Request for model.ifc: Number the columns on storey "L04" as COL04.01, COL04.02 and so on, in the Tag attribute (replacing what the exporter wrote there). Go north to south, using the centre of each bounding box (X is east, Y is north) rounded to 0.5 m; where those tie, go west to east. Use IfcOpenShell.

First a look at what the model holds.

```python
import ifcopenshell
import ifcopenshell.util.element
import ifcopenshell.util.placement

model = ifcopenshell.open("model.ifc")
print(model.schema)
storey = next(s for s in model.by_type("IfcBuildingStorey") if s.Name == "L04")
columns = [e for e in ifcopenshell.util.element.get_decomposition(storey) if e.is_a("IfcColumn")]
for e in sorted(columns, key=lambda e: e.id()):
    origin = ifcopenshell.util.placement.get_local_placement(e.ObjectPlacement)[:3, 3]
    print(e.id(), e.Tag, e.Name, origin.round(2) + 0.0, sep=" | ")
```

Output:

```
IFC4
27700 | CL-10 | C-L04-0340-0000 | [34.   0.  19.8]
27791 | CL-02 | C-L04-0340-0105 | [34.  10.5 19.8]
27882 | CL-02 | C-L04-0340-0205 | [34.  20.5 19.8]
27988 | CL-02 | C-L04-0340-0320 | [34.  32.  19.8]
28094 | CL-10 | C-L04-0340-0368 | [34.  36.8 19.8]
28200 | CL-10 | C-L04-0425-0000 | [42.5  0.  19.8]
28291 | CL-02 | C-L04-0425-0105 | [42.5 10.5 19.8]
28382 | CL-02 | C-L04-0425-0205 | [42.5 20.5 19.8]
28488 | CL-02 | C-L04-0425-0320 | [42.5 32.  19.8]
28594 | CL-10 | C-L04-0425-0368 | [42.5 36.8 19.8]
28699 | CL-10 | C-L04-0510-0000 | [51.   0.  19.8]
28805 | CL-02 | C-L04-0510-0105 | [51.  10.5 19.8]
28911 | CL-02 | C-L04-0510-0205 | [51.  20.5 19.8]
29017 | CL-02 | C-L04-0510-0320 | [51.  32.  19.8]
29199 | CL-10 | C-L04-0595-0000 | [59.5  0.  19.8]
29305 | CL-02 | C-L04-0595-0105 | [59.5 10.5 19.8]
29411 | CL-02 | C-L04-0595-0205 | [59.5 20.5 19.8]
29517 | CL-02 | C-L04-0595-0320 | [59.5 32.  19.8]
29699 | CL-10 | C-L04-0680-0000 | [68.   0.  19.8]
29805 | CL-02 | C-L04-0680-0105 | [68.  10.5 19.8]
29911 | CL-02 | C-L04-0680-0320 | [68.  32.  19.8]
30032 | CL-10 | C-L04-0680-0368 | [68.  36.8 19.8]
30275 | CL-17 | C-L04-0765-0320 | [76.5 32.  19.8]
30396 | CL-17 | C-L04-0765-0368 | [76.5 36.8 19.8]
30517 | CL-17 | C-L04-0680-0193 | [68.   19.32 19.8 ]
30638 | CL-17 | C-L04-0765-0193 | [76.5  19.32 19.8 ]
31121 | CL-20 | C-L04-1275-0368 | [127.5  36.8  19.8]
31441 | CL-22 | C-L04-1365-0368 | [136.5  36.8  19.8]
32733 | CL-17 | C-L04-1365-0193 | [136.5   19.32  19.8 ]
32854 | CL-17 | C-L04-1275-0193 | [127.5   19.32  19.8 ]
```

```python
import ifcopenshell
import ifcopenshell.geom
import ifcopenshell.util.element
import ifcopenshell.util.shape

model = ifcopenshell.open("model.ifc")
settings = ifcopenshell.geom.settings()
settings.set("use-world-coords", True)


def centre(element):
    shape = ifcopenshell.geom.create_shape(settings, element)
    return ifcopenshell.util.shape.get_bbox_centroid(shape.geometry)


storey = next(s for s in model.by_type("IfcBuildingStorey") if s.Name == "L04")
columns = [e for e in ifcopenshell.util.element.get_decomposition(storey) if e.is_a("IfcColumn")]

# Insertion points can sit at a corner or the storey origin, so sort by the geometry (in metres).
centres = {e: centre(e) for e in columns}
columns.sort(key=lambda e: (-round(centres[e][1] / 0.5), centres[e][0]))

for i, e in enumerate(columns, start=1):
    number = f"COL04.{i:02d}"
    e.Tag = number
    print(e.id(), number)

model.write("model_updated.ifc")
```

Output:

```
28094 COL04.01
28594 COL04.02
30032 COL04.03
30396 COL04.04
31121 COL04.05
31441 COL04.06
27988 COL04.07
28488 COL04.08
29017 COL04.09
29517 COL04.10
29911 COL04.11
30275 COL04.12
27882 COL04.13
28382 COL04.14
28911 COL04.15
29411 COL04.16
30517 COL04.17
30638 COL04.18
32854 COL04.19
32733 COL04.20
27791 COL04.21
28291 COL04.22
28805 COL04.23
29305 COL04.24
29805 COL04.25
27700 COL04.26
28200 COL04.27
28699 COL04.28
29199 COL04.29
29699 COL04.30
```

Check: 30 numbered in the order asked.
